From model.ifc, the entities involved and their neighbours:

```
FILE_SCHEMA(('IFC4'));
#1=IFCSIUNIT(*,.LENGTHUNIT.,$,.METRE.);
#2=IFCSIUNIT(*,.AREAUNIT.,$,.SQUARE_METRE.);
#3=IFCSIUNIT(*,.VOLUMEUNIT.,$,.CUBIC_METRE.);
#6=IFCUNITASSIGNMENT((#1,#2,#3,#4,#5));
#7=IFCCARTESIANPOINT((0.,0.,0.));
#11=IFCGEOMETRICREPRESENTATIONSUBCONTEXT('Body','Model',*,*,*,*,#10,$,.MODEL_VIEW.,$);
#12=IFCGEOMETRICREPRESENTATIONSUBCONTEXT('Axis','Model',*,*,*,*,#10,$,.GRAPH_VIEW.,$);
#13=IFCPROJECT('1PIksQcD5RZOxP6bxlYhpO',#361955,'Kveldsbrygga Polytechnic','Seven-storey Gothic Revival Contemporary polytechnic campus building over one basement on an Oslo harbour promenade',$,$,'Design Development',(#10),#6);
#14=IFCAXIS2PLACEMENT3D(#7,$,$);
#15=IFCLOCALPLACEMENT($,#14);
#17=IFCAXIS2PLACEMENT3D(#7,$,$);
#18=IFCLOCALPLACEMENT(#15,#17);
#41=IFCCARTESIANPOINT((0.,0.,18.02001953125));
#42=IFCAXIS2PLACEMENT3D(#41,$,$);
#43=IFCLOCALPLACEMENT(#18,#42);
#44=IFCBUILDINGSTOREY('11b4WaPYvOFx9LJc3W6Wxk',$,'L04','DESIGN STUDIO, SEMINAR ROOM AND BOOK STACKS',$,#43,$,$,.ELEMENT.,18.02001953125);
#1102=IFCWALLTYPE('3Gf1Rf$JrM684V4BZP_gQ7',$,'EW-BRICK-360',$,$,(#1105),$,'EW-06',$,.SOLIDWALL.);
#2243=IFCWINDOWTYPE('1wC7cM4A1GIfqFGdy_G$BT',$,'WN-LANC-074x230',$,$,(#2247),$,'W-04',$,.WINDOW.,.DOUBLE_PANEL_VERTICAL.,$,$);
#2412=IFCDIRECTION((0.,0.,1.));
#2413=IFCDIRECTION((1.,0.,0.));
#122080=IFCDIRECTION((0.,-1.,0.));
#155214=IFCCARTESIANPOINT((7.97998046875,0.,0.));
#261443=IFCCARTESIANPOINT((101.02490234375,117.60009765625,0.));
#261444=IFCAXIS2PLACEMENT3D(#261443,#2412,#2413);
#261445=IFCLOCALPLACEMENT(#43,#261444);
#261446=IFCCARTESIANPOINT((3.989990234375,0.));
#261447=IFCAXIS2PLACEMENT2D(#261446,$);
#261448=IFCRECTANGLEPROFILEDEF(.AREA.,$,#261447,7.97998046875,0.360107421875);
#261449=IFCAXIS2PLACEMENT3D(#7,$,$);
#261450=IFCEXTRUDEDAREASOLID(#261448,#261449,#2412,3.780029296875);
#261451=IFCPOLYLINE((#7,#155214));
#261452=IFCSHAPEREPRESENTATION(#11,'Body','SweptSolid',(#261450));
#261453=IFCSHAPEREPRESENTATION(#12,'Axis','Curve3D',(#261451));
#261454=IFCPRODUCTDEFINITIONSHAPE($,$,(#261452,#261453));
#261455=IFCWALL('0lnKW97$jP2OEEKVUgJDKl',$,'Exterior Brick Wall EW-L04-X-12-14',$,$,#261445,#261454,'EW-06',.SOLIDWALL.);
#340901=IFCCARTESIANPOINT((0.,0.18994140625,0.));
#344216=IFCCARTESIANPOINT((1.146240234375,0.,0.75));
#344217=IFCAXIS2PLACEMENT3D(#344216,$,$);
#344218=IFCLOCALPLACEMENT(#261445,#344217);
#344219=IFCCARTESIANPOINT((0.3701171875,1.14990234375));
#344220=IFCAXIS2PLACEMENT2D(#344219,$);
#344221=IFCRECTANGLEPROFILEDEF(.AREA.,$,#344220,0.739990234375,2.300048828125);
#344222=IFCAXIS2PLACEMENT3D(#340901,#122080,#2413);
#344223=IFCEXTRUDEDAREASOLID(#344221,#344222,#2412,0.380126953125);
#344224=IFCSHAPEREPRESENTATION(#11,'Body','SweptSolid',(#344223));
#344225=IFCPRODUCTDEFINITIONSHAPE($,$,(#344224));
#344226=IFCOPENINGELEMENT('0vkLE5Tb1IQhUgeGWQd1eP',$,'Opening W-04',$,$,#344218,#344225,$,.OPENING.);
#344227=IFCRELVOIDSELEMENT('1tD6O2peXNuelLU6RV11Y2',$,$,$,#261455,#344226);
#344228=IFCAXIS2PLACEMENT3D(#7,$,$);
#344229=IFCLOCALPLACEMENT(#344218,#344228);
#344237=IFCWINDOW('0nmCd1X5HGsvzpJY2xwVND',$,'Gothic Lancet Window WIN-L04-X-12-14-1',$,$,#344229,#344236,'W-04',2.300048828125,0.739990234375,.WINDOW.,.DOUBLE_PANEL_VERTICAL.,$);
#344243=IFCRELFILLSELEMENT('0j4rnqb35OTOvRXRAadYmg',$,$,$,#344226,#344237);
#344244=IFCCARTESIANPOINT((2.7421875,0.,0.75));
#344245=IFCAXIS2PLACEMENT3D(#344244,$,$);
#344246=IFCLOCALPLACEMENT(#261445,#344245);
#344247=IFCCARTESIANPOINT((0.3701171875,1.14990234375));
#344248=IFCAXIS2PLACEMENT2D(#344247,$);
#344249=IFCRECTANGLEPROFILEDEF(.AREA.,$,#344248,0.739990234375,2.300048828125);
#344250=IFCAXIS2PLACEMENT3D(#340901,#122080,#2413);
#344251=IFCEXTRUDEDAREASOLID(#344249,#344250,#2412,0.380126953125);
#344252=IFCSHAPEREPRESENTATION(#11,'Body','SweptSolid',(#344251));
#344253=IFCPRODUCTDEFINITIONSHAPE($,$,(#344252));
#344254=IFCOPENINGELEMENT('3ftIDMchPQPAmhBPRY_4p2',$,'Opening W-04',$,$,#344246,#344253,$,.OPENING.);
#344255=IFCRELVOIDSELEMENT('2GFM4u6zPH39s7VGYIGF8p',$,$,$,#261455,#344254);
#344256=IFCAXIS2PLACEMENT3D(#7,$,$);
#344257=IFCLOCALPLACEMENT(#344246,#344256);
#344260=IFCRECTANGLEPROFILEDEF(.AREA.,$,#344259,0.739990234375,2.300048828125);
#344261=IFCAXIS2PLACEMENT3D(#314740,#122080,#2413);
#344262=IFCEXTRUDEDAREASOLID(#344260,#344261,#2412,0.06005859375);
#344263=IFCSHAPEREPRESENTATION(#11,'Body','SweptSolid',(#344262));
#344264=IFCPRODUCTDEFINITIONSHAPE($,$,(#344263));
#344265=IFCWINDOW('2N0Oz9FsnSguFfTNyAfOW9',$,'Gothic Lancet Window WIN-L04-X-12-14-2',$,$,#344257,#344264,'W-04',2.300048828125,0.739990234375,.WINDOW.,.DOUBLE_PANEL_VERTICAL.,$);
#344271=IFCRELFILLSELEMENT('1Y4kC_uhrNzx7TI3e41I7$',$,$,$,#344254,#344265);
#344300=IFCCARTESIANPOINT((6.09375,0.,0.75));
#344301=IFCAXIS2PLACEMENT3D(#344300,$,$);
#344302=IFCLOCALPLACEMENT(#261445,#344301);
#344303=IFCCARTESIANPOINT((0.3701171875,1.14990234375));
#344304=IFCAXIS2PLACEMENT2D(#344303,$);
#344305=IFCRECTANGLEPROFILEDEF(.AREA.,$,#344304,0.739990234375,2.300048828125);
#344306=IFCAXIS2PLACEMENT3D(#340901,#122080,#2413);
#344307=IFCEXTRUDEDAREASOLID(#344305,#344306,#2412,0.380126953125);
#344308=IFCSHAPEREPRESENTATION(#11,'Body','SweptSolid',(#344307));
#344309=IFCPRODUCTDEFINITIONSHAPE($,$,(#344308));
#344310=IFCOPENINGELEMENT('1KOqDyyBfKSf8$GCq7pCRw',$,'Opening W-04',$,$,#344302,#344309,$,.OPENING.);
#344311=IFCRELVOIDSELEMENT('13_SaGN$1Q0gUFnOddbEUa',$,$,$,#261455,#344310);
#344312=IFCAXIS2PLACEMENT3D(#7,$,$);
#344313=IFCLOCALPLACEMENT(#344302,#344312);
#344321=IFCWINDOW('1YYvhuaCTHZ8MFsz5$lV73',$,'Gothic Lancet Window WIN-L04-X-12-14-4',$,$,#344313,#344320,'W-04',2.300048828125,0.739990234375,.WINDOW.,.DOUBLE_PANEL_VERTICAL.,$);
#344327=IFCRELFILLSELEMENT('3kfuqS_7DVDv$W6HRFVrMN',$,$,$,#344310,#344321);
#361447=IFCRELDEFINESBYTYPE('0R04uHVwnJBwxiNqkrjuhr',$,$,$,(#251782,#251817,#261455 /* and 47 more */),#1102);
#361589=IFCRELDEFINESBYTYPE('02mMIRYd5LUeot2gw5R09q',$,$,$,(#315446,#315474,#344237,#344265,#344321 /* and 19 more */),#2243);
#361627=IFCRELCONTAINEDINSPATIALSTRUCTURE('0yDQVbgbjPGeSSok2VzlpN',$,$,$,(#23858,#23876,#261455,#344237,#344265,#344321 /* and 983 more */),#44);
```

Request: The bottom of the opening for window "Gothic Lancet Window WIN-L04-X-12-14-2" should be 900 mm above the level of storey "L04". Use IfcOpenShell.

```python
import numpy as np
import ifcopenshell
import ifcopenshell.api.geometry
import ifcopenshell.geom
import ifcopenshell.util.element
import ifcopenshell.util.placement
import ifcopenshell.util.shape
import ifcopenshell.util.unit

model = ifcopenshell.open("model.ifc")
unit_scale = ifcopenshell.util.unit.calculate_unit_scale(model)

window = model.by_guid("2N0Oz9FsnSguFfTNyAfOW9")
opening = window.FillsVoids[0].RelatingOpeningElement
storey = ifcopenshell.util.element.get_container(window, ifc_class="IfcBuildingStorey")
level = ifcopenshell.util.placement.get_local_placement(storey.ObjectPlacement)[2, 3]

# The opening's origin need not be at the sill, so measure its lowest point.
shape = ifcopenshell.geom.create_shape(ifcopenshell.geom.settings(), opening)
bottom = ifcopenshell.util.shape.get_shape_bottom_elevation(shape, shape.geometry) / unit_scale
dz = level + 0.9 / unit_scale - bottom

shift = np.array([0.0, 0.0, dz])
# The window is placed relative to its opening, so it follows when the opening moves.
matrix = ifcopenshell.util.placement.get_local_placement(opening.ObjectPlacement)
matrix[:3, 3] += shift
ifcopenshell.api.geometry.edit_object_placement(
    model, product=opening, matrix=matrix, is_si=False, should_transform_children=True
)

print(f"moved by {dz * unit_scale:+.3f} m")

model.write("model_v2.ifc")
```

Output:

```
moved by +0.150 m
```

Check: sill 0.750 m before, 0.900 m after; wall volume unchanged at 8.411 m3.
